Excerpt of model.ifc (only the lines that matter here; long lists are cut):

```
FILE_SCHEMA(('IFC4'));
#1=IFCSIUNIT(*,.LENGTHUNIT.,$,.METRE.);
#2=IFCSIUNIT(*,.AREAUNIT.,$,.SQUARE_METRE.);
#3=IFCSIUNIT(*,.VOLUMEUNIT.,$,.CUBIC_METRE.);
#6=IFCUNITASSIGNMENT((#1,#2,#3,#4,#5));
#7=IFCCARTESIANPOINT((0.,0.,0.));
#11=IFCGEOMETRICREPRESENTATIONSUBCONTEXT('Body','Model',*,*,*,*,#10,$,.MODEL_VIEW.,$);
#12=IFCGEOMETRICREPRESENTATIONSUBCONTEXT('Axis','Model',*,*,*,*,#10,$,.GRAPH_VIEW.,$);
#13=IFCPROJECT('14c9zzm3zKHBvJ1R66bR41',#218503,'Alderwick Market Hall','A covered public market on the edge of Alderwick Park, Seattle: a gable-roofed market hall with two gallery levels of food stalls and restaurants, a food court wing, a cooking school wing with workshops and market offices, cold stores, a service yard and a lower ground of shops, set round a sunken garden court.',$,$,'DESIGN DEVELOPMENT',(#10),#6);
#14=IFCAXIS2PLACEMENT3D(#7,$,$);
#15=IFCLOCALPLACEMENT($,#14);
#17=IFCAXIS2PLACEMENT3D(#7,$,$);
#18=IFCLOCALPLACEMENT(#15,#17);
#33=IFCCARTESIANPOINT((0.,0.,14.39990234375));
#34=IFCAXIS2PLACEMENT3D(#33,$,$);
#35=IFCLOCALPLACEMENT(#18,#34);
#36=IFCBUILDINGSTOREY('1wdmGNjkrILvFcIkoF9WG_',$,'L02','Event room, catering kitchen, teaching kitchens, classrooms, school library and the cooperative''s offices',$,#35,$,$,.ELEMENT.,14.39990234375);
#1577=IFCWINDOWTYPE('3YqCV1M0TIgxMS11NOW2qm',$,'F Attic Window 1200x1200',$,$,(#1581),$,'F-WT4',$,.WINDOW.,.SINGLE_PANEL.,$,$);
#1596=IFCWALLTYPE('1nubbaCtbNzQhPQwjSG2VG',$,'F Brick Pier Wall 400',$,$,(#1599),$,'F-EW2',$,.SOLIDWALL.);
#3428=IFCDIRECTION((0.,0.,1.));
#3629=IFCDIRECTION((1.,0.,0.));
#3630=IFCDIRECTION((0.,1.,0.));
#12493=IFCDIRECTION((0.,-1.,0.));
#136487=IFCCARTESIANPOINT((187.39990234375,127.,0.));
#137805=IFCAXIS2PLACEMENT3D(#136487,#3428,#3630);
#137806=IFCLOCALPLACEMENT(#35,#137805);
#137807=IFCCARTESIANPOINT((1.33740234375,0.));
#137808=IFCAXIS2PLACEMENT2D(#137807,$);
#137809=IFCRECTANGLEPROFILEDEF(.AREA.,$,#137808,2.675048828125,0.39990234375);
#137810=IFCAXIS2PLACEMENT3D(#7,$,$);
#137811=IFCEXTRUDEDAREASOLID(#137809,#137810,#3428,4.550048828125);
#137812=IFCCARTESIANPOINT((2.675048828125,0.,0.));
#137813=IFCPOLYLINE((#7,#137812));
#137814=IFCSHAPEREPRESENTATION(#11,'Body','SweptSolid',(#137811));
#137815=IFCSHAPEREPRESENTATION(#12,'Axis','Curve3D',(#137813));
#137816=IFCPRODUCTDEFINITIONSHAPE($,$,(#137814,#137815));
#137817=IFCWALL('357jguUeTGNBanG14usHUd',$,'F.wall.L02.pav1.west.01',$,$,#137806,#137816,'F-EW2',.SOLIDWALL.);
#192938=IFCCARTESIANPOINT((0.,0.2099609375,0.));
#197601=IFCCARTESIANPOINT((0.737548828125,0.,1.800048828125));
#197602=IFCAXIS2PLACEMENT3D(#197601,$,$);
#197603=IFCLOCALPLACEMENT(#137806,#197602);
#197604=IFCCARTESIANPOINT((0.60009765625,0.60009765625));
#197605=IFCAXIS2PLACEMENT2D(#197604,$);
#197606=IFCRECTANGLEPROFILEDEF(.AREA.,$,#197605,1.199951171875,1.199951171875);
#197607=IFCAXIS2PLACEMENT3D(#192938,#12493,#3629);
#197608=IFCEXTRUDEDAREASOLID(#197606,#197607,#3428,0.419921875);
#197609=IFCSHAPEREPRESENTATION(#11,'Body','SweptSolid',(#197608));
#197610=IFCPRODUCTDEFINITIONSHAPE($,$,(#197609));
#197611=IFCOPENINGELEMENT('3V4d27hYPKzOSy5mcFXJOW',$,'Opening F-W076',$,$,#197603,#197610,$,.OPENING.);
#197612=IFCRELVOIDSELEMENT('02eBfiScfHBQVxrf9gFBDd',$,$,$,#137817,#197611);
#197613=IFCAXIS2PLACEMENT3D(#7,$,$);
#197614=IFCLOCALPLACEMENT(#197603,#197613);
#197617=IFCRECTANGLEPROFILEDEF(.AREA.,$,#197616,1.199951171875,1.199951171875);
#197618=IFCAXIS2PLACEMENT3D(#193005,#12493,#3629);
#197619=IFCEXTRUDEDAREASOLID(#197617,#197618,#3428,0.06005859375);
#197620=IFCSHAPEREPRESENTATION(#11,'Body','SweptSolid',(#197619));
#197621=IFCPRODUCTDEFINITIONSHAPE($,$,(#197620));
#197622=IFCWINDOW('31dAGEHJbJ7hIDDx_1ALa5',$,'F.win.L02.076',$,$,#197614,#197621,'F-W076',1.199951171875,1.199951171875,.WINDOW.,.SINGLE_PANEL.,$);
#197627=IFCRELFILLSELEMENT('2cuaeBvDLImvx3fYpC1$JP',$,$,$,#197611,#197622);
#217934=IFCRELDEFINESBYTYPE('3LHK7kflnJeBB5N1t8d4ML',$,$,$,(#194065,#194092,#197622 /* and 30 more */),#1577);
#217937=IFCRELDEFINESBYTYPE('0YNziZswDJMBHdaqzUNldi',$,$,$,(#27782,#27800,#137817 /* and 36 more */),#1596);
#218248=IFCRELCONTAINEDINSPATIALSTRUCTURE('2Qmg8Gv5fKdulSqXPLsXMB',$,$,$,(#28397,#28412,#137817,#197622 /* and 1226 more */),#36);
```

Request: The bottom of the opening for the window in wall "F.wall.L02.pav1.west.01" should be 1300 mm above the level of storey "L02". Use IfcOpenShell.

```python
import numpy as np
import ifcopenshell
import ifcopenshell.api.geometry
import ifcopenshell.geom
import ifcopenshell.util.element
import ifcopenshell.util.placement
import ifcopenshell.util.shape
import ifcopenshell.util.unit

model = ifcopenshell.open("model.ifc")
unit_scale = ifcopenshell.util.unit.calculate_unit_scale(model)

window = model.by_guid("31dAGEHJbJ7hIDDx_1ALa5")
opening = window.FillsVoids[0].RelatingOpeningElement
storey = ifcopenshell.util.element.get_container(window, ifc_class="IfcBuildingStorey")
level = ifcopenshell.util.placement.get_local_placement(storey.ObjectPlacement)[2, 3]

# The opening's origin need not be at the sill, so measure its lowest point.
shape = ifcopenshell.geom.create_shape(ifcopenshell.geom.settings(), opening)
bottom = ifcopenshell.util.shape.get_shape_bottom_elevation(shape, shape.geometry) / unit_scale
dz = level + 1.3 / unit_scale - bottom

shift = np.array([0.0, 0.0, dz])
# The window is placed relative to its opening, so it follows when the opening moves.
matrix = ifcopenshell.util.placement.get_local_placement(opening.ObjectPlacement)
matrix[:3, 3] += shift
ifcopenshell.api.geometry.edit_object_placement(
    model, product=opening, matrix=matrix, is_si=False, should_transform_children=True
)

print(f"moved by {dz * unit_scale:+.3f} m")

model.write("model_updated.ifc")
```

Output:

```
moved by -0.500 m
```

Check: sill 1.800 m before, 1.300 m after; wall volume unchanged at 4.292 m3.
